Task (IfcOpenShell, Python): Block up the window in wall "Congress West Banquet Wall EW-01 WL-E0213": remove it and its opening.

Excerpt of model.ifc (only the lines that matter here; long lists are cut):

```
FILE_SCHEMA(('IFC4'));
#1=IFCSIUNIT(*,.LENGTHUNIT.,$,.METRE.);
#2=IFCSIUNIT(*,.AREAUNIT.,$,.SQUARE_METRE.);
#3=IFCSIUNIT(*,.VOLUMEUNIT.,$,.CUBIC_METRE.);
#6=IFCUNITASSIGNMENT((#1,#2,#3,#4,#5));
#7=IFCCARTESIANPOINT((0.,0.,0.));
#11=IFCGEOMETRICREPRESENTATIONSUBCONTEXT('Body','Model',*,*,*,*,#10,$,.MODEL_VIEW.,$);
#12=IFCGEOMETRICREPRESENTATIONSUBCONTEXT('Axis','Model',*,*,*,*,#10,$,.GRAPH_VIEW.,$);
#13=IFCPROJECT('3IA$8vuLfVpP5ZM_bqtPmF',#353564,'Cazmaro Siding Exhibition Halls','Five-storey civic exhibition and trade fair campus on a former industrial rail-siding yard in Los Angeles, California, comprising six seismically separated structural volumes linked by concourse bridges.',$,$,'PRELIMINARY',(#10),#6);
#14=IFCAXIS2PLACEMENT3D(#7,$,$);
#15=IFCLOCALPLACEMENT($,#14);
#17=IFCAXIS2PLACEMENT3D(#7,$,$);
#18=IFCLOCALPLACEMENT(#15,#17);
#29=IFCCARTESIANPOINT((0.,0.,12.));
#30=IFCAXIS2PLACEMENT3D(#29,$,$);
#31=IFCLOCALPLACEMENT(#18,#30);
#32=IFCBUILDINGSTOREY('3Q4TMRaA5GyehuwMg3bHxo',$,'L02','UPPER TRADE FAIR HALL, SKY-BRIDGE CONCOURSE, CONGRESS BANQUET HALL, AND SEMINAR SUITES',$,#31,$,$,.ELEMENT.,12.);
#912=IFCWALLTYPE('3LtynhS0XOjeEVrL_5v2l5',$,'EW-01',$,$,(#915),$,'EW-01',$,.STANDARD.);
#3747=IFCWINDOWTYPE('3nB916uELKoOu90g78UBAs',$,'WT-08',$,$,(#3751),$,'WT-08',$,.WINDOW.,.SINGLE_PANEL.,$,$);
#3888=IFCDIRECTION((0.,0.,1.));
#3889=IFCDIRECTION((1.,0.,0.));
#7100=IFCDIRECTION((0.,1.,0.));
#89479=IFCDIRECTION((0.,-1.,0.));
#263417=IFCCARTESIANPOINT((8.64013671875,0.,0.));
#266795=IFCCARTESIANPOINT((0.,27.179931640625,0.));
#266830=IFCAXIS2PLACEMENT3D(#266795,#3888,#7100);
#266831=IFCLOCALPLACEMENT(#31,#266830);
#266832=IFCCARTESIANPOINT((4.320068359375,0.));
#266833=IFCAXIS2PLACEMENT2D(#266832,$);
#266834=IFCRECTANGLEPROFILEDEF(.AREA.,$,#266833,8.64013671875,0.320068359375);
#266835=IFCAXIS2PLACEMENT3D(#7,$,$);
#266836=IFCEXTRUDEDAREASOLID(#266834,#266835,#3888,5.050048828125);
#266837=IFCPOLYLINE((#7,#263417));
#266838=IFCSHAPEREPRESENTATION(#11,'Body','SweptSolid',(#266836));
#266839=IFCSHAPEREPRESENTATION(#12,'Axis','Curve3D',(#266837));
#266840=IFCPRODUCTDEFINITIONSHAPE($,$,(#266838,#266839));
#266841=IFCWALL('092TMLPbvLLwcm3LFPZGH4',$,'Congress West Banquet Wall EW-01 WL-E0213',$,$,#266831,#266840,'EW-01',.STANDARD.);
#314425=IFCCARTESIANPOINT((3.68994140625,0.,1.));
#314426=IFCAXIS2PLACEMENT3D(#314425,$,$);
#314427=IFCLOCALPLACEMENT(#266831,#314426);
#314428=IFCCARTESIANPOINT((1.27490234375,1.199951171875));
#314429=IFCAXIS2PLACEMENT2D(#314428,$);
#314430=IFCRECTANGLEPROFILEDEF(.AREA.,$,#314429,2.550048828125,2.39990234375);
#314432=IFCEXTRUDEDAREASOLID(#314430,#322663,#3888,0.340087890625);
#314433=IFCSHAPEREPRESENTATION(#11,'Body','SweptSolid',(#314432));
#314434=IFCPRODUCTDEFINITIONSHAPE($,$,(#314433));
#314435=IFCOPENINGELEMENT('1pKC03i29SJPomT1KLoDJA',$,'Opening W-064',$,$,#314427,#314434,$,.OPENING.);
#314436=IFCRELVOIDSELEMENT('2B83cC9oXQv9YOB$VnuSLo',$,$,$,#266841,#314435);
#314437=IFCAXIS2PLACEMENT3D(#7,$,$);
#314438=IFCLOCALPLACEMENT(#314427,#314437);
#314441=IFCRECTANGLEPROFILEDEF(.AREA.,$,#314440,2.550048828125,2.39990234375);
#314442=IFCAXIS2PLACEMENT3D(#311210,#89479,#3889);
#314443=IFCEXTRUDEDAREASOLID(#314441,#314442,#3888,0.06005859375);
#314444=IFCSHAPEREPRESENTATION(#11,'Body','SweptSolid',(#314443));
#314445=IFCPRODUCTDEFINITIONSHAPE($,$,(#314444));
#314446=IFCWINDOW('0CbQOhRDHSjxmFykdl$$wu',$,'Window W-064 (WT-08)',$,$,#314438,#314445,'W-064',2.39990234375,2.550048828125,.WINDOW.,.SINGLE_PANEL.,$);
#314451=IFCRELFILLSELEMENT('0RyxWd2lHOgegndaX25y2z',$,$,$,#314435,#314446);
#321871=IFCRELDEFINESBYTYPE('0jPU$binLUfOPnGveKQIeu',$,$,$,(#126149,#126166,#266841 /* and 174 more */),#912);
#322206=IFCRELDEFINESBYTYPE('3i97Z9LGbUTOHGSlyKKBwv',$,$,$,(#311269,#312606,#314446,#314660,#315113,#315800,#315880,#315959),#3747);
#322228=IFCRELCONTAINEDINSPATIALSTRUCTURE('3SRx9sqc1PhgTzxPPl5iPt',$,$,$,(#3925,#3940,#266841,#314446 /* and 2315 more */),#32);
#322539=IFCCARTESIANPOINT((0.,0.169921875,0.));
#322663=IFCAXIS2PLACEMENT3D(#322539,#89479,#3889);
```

```python
import ifcopenshell
import ifcopenshell.api.feature
import ifcopenshell.api.root
import ifcopenshell.geom
import ifcopenshell.util.shape

model = ifcopenshell.open("model.ifc")
settings = ifcopenshell.geom.settings()


def volume(element):
    """Net volume in cubic metres, openings subtracted."""
    shape = ifcopenshell.geom.create_shape(settings, element)
    return ifcopenshell.util.shape.get_volume(shape.geometry)


window = model.by_guid("0CbQOhRDHSjxmFykdl$$wu")
opening = window.FillsVoids[0].RelatingOpeningElement
wall = opening.VoidsElements[0].RelatingBuildingElement
before = volume(wall)

ifcopenshell.api.root.remove_product(model, product=window)
ifcopenshell.api.feature.remove_feature(model, feature=opening)

after = volume(wall)

print(f"wall volume {before:.3f} -> {after:.3f} m3")

model.write("model_edited.ifc")
```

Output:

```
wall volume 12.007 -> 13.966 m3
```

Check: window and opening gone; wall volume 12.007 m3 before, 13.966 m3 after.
